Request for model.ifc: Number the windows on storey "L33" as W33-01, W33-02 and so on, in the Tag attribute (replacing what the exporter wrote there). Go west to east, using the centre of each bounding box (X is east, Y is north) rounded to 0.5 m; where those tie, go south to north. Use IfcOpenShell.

First a look at what the model holds.

```python
import ifcopenshell
import ifcopenshell.util.element
import ifcopenshell.util.placement

model = ifcopenshell.open("model.ifc")
print(model.schema)
storey = next(s for s in model.by_type("IfcBuildingStorey") if s.Name == "L33")
windows = [e for e in ifcopenshell.util.element.get_decomposition(storey) if e.is_a("IfcWindow")]
for e in sorted(windows, key=lambda e: e.id()):
    origin = ifcopenshell.util.placement.get_local_placement(e.ObjectPlacement)[:3, 3]
    print(e.id(), e.Tag, e.Name, origin.round(2) + 0.0, sep=" | ")
```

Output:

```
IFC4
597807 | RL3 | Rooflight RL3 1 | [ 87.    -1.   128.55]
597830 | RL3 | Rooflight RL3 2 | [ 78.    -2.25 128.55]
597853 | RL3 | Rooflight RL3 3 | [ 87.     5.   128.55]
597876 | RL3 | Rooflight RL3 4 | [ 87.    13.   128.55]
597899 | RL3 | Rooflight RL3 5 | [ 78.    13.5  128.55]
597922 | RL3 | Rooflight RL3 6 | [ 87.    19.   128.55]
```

```python
import ifcopenshell
import ifcopenshell.geom
import ifcopenshell.util.element
import ifcopenshell.util.shape

model = ifcopenshell.open("model.ifc")
settings = ifcopenshell.geom.settings()
settings.set("use-world-coords", True)


def centre(element):
    shape = ifcopenshell.geom.create_shape(settings, element)
    return ifcopenshell.util.shape.get_bbox_centroid(shape.geometry)


storey = next(s for s in model.by_type("IfcBuildingStorey") if s.Name == "L33")
windows = [e for e in ifcopenshell.util.element.get_decomposition(storey) if e.is_a("IfcWindow")]

# Insertion points can sit at a corner or the storey origin, so sort by the geometry (in metres).
centres = {e: centre(e) for e in windows}
windows.sort(key=lambda e: (round(centres[e][0] / 0.5), centres[e][1]))

for i, e in enumerate(windows, start=1):
    number = f"W33-{i:02d}"
    e.Tag = number
    print(e.id(), number)

model.write("model-out.ifc")
```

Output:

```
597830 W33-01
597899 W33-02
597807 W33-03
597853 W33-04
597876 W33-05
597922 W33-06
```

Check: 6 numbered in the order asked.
